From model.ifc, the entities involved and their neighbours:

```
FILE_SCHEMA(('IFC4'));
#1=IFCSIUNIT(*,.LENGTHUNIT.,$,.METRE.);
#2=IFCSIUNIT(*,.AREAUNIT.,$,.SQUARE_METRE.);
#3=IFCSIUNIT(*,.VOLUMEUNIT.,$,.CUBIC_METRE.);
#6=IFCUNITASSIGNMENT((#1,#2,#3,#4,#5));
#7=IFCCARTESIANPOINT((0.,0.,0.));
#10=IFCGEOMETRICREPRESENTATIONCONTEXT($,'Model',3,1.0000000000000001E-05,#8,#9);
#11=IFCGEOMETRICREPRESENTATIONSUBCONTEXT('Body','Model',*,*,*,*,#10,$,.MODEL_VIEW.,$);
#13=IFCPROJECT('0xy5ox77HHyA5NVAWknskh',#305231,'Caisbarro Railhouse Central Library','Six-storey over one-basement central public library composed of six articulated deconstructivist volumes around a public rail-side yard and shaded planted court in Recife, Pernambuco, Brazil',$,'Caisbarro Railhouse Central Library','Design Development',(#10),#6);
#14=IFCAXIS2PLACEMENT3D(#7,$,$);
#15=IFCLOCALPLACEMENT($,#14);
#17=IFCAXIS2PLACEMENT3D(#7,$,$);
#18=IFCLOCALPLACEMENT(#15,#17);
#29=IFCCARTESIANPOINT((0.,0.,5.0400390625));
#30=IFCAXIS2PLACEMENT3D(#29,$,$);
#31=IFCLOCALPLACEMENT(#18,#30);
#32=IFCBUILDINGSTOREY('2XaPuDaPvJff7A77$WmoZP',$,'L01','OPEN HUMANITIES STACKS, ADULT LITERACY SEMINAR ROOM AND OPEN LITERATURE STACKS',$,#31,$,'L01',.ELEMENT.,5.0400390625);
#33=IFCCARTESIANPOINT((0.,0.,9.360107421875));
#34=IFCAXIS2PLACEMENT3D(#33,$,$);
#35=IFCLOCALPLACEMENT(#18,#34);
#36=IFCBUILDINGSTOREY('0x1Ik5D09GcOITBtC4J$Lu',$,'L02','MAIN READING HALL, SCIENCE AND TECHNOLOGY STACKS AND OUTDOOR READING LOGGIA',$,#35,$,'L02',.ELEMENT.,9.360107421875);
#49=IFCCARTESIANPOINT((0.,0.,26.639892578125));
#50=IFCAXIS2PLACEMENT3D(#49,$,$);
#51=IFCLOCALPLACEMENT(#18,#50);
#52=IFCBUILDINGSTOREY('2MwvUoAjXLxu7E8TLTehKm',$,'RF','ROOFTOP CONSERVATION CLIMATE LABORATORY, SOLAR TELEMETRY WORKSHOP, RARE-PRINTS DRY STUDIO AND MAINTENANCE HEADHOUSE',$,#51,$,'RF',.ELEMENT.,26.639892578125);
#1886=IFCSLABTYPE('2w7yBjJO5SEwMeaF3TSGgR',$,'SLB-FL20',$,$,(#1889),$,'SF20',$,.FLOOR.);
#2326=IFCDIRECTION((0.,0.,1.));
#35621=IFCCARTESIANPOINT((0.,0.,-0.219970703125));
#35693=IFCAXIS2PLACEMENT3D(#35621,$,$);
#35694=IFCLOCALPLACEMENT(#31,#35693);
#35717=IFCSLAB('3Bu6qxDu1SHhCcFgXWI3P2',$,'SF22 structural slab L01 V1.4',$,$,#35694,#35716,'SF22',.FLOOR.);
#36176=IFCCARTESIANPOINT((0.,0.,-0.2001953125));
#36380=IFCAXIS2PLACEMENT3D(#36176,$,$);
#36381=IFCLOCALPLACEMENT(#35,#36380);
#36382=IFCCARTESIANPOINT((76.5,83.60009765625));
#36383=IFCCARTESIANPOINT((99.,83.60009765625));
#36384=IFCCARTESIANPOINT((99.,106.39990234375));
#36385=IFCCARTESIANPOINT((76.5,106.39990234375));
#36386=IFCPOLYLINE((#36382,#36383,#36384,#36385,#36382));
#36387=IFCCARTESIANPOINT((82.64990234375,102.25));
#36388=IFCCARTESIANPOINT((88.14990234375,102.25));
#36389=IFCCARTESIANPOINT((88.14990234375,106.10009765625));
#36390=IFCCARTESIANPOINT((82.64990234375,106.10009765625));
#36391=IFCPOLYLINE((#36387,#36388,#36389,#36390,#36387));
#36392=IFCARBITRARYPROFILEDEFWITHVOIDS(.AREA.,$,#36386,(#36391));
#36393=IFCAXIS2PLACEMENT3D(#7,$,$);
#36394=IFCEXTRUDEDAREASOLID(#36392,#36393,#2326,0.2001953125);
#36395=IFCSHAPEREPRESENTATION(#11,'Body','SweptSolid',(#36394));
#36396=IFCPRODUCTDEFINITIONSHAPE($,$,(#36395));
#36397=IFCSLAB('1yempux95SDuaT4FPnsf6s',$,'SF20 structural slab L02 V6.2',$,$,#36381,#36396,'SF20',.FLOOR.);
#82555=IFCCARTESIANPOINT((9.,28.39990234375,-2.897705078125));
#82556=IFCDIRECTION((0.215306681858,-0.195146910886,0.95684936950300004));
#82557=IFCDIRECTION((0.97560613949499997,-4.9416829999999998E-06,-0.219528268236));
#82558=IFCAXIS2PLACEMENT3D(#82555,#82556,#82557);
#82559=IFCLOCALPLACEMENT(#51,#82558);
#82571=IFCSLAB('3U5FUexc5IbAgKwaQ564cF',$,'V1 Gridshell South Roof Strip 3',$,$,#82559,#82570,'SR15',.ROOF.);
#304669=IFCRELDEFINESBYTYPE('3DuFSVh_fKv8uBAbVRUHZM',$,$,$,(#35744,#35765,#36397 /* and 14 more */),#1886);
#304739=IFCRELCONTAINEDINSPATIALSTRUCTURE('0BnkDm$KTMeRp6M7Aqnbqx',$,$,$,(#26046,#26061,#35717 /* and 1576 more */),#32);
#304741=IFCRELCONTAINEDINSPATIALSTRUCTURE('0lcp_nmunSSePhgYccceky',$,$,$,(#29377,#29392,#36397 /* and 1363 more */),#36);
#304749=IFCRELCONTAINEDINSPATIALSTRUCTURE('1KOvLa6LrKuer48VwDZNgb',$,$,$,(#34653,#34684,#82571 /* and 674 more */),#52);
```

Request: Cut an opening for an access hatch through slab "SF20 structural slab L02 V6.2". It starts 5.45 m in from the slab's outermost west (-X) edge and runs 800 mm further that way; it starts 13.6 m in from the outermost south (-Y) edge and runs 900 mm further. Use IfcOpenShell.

```python
import numpy as np
import ifcopenshell
import ifcopenshell.api.feature
import ifcopenshell.api.geometry
import ifcopenshell.api.root
import ifcopenshell.geom
import ifcopenshell.util.placement
import ifcopenshell.util.representation
import ifcopenshell.util.shape
import ifcopenshell.util.unit

model = ifcopenshell.open("model.ifc")
unit_scale = ifcopenshell.util.unit.calculate_unit_scale(model)
settings = ifcopenshell.geom.settings()


def volume(element):
    """Net volume in cubic metres, openings subtracted."""
    shape = ifcopenshell.geom.create_shape(settings, element)
    return ifcopenshell.util.shape.get_volume(shape.geometry)


slab = model.by_guid("1yempux95SDuaT4FPnsf6s")
before = volume(slab)

# Extent in the slab's own axes, in metres. The edges named are its -X and -Y sides.
slab_shape = ifcopenshell.geom.create_shape(settings, slab)
vertices = ifcopenshell.util.shape.get_vertices(slab_shape.geometry)
x_min, y_min, bottom = vertices.min(axis=0)
top = vertices[:, 2].max()

opening = ifcopenshell.api.root.create_entity(model, ifc_class="IfcOpeningElement", name="Access hatch opening", predefined_type="OPENING")
context = ifcopenshell.util.representation.get_context(model, "Model", "Body", "MODEL_VIEW")
width, depth = 0.8, 0.9
outline = [(0.0, 0.0), (width, 0.0), (width, depth), (0.0, depth), (0.0, 0.0)]
# Overshoot both faces by 50 mm so the cut is clean.
shape = ifcopenshell.api.geometry.add_slab_representation(
    model, context=context, depth=top - bottom + 0.1, polyline=outline
)
ifcopenshell.api.geometry.assign_representation(model, product=opening, representation=shape)

matrix = ifcopenshell.util.placement.get_local_placement(slab.ObjectPlacement)
matrix[:, 3] = matrix @ np.append(np.array([x_min + 5.45, y_min + 13.6, bottom - 0.05]) / unit_scale, 1.0)
ifcopenshell.api.geometry.edit_object_placement(model, product=opening, matrix=matrix, is_si=False)
ifcopenshell.api.feature.add_feature(model, feature=opening, element=slab)

after = volume(slab)

print(f"slab volume {before:.3f} -> {after:.3f} m3")

model.write("model_v2.ifc")
```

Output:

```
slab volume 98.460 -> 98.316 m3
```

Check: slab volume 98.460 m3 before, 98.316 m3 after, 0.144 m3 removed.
